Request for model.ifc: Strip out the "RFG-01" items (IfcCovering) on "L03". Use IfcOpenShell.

First a look at what the model holds.

```python
import ifcopenshell
import ifcopenshell.util.element

model = ifcopenshell.open("model.ifc")
print(model.schema)
storey = next(s for s in model.by_type("IfcBuildingStorey") if s.Name == "L03")
coverings = [e for e in ifcopenshell.util.element.get_decomposition(storey) if e.is_a("IfcCovering")]
seen = {}
for e in coverings:
    element_type = ifcopenshell.util.element.get_type(e)
    name = element_type.Name if element_type not in (None, e) else None
    seen[name] = seen.get(name, 0) + 1
for name, count in sorted(seen.items(), key=str):
    print(count, "x", name)
```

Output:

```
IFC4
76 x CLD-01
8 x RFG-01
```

```python
import ifcopenshell
import ifcopenshell.api.root
import ifcopenshell.util.element

model = ifcopenshell.open("model.ifc")

storey = next(s for s in model.by_type("IfcBuildingStorey") if s.Name == "L03")
coverings = [e for e in ifcopenshell.util.element.get_decomposition(storey) if e.is_a("IfcCovering")]
targets = [e for e in coverings if (t := ifcopenshell.util.element.get_type(e)) not in (None, e) and t.Name == "RFG-01"]

for e in targets:
    ifcopenshell.api.root.remove_product(model, product=e)
print(len(targets), "removed")

model.write("model_edited.ifc")
```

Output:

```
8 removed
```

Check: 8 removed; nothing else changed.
